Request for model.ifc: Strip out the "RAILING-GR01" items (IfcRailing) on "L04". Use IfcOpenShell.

First a look at what the model holds.

```python
import ifcopenshell
import ifcopenshell.util.element

model = ifcopenshell.open("model.ifc")
print(model.schema)
storey = next(s for s in model.by_type("IfcBuildingStorey") if s.Name == "L04")
railings = [e for e in ifcopenshell.util.element.get_decomposition(storey) if e.is_a("IfcRailing")]
seen = {}
for e in railings:
    element_type = ifcopenshell.util.element.get_type(e)
    name = element_type.Name if element_type not in (None, e) else None
    seen[name] = seen.get(name, 0) + 1
for name, count in sorted(seen.items(), key=str):
    print(count, "x", name)
```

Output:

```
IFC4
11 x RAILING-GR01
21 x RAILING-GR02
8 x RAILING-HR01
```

```python
import ifcopenshell
import ifcopenshell.api.root
import ifcopenshell.util.element

model = ifcopenshell.open("model.ifc")

storey = next(s for s in model.by_type("IfcBuildingStorey") if s.Name == "L04")
railings = [e for e in ifcopenshell.util.element.get_decomposition(storey) if e.is_a("IfcRailing")]
targets = [e for e in railings if (t := ifcopenshell.util.element.get_type(e)) not in (None, e) and t.Name == "RAILING-GR01"]

for e in targets:
    ifcopenshell.api.root.remove_product(model, product=e)
print(len(targets), "removed")

model.write("model_edited.ifc")
```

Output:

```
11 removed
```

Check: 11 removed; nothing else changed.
